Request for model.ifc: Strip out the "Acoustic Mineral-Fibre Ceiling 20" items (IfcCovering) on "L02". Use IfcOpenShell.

First a look at what the model holds.

```python
import ifcopenshell
import ifcopenshell.util.element

model = ifcopenshell.open("model.ifc")
print(model.schema)
storey = next(s for s in model.by_type("IfcBuildingStorey") if s.Name == "L02")
coverings = [e for e in ifcopenshell.util.element.get_decomposition(storey) if e.is_a("IfcCovering")]
seen = {}
for e in coverings:
    element_type = ifcopenshell.util.element.get_type(e)
    name = element_type.Name if element_type not in (None, e) else None
    seen[name] = seen.get(name, 0) + 1
for name, count in sorted(seen.items(), key=str):
    print(count, "x", name)
```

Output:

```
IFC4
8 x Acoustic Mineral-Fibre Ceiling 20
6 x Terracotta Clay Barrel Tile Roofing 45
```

```python
import ifcopenshell
import ifcopenshell.api.root
import ifcopenshell.util.element

model = ifcopenshell.open("model.ifc")

storey = next(s for s in model.by_type("IfcBuildingStorey") if s.Name == "L02")
coverings = [e for e in ifcopenshell.util.element.get_decomposition(storey) if e.is_a("IfcCovering")]
targets = [e for e in coverings if (t := ifcopenshell.util.element.get_type(e)) not in (None, e) and t.Name == "Acoustic Mineral-Fibre Ceiling 20"]

for e in targets:
    ifcopenshell.api.root.remove_product(model, product=e)
print(len(targets), "removed")

model.write("model_rev.ifc")
```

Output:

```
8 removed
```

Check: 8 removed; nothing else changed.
